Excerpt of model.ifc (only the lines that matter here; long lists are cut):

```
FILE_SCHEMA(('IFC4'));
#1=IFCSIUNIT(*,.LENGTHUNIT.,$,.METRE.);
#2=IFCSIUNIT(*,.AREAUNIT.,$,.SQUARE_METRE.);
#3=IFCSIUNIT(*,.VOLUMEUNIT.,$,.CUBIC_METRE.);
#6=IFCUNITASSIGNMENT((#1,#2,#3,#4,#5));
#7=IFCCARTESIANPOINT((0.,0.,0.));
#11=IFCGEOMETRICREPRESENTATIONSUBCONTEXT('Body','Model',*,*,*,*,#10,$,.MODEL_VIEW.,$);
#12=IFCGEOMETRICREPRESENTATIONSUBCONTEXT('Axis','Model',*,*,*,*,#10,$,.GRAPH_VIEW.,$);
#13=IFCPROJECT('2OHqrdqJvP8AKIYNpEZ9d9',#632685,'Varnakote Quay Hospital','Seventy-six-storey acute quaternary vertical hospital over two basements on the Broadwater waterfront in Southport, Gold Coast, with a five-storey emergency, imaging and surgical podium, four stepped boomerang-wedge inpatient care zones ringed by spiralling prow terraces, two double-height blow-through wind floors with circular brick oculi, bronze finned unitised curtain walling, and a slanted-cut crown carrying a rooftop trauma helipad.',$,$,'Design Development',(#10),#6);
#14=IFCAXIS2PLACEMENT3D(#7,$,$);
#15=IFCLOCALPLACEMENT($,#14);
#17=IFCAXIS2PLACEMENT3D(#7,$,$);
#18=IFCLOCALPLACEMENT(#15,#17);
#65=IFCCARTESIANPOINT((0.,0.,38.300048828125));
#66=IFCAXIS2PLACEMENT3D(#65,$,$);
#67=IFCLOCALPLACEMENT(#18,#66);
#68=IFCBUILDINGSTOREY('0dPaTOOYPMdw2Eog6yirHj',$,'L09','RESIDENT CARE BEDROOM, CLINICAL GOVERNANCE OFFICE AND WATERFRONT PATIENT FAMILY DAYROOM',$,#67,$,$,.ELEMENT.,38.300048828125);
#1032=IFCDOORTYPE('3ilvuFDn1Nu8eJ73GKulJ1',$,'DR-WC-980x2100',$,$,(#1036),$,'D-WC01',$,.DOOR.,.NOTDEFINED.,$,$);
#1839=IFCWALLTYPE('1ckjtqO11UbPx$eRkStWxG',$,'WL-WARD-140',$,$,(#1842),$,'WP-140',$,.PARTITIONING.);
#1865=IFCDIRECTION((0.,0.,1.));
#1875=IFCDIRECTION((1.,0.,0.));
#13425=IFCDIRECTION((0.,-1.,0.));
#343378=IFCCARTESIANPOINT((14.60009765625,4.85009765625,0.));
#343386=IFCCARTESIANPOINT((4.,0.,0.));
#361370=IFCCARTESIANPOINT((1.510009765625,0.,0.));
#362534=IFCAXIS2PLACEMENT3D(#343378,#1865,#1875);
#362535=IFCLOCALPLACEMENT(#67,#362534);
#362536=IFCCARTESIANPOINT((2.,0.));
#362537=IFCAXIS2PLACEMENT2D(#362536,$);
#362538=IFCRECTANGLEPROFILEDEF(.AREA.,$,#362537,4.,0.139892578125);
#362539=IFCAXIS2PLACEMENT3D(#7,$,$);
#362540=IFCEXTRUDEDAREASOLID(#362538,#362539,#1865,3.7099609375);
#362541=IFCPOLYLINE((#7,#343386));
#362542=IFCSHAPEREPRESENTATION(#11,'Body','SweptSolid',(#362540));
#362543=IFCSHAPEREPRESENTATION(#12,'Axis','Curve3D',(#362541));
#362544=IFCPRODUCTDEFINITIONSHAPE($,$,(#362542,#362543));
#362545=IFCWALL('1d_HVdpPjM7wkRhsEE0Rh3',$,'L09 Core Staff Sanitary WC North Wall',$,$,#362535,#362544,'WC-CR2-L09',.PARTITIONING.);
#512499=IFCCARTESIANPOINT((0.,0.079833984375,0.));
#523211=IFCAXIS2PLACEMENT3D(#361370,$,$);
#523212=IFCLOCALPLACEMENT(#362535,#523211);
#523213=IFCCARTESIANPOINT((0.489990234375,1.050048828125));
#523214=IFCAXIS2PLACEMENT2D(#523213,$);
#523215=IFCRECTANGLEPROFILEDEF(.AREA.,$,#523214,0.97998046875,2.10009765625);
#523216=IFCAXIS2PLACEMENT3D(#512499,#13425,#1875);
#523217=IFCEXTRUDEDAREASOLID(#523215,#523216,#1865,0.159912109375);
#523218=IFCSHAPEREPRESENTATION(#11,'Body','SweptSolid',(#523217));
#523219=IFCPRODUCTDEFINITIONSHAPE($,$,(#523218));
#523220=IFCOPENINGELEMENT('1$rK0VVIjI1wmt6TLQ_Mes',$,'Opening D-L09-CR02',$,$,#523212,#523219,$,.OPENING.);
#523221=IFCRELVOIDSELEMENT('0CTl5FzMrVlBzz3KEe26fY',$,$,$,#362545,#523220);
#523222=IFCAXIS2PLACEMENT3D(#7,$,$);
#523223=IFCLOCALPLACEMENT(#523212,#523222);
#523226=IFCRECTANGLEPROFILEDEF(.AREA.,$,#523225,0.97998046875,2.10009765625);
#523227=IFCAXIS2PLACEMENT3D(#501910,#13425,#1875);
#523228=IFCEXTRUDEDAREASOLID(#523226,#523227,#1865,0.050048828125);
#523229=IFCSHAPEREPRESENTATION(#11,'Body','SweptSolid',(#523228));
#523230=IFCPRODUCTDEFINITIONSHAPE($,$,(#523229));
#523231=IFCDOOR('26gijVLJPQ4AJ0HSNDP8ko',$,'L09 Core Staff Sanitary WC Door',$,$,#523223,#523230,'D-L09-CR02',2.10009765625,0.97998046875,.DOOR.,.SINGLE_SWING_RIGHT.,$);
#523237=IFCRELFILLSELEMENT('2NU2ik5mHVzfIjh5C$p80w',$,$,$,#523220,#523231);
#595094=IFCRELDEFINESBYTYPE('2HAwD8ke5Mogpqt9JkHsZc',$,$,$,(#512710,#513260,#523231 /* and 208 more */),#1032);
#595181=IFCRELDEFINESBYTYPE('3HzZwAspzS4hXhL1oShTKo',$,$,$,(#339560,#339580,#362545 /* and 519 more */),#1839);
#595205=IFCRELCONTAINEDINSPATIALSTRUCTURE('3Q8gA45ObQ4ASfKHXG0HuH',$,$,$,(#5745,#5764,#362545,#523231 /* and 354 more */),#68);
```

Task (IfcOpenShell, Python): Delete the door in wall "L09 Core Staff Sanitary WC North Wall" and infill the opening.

```python
import ifcopenshell
import ifcopenshell.api.feature
import ifcopenshell.api.root
import ifcopenshell.geom
import ifcopenshell.util.shape

model = ifcopenshell.open("model.ifc")
settings = ifcopenshell.geom.settings()


def volume(element):
    """Net volume in cubic metres, openings subtracted."""
    shape = ifcopenshell.geom.create_shape(settings, element)
    return ifcopenshell.util.shape.get_volume(shape.geometry)


door = model.by_guid("26gijVLJPQ4AJ0HSNDP8ko")
opening = door.FillsVoids[0].RelatingOpeningElement
wall = opening.VoidsElements[0].RelatingBuildingElement
before = volume(wall)

ifcopenshell.api.root.remove_product(model, product=door)
ifcopenshell.api.feature.remove_feature(model, feature=opening)

after = volume(wall)

print(f"wall volume {before:.3f} -> {after:.3f} m3")

model.write("model_updated.ifc")
```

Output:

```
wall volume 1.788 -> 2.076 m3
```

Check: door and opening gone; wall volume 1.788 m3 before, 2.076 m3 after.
